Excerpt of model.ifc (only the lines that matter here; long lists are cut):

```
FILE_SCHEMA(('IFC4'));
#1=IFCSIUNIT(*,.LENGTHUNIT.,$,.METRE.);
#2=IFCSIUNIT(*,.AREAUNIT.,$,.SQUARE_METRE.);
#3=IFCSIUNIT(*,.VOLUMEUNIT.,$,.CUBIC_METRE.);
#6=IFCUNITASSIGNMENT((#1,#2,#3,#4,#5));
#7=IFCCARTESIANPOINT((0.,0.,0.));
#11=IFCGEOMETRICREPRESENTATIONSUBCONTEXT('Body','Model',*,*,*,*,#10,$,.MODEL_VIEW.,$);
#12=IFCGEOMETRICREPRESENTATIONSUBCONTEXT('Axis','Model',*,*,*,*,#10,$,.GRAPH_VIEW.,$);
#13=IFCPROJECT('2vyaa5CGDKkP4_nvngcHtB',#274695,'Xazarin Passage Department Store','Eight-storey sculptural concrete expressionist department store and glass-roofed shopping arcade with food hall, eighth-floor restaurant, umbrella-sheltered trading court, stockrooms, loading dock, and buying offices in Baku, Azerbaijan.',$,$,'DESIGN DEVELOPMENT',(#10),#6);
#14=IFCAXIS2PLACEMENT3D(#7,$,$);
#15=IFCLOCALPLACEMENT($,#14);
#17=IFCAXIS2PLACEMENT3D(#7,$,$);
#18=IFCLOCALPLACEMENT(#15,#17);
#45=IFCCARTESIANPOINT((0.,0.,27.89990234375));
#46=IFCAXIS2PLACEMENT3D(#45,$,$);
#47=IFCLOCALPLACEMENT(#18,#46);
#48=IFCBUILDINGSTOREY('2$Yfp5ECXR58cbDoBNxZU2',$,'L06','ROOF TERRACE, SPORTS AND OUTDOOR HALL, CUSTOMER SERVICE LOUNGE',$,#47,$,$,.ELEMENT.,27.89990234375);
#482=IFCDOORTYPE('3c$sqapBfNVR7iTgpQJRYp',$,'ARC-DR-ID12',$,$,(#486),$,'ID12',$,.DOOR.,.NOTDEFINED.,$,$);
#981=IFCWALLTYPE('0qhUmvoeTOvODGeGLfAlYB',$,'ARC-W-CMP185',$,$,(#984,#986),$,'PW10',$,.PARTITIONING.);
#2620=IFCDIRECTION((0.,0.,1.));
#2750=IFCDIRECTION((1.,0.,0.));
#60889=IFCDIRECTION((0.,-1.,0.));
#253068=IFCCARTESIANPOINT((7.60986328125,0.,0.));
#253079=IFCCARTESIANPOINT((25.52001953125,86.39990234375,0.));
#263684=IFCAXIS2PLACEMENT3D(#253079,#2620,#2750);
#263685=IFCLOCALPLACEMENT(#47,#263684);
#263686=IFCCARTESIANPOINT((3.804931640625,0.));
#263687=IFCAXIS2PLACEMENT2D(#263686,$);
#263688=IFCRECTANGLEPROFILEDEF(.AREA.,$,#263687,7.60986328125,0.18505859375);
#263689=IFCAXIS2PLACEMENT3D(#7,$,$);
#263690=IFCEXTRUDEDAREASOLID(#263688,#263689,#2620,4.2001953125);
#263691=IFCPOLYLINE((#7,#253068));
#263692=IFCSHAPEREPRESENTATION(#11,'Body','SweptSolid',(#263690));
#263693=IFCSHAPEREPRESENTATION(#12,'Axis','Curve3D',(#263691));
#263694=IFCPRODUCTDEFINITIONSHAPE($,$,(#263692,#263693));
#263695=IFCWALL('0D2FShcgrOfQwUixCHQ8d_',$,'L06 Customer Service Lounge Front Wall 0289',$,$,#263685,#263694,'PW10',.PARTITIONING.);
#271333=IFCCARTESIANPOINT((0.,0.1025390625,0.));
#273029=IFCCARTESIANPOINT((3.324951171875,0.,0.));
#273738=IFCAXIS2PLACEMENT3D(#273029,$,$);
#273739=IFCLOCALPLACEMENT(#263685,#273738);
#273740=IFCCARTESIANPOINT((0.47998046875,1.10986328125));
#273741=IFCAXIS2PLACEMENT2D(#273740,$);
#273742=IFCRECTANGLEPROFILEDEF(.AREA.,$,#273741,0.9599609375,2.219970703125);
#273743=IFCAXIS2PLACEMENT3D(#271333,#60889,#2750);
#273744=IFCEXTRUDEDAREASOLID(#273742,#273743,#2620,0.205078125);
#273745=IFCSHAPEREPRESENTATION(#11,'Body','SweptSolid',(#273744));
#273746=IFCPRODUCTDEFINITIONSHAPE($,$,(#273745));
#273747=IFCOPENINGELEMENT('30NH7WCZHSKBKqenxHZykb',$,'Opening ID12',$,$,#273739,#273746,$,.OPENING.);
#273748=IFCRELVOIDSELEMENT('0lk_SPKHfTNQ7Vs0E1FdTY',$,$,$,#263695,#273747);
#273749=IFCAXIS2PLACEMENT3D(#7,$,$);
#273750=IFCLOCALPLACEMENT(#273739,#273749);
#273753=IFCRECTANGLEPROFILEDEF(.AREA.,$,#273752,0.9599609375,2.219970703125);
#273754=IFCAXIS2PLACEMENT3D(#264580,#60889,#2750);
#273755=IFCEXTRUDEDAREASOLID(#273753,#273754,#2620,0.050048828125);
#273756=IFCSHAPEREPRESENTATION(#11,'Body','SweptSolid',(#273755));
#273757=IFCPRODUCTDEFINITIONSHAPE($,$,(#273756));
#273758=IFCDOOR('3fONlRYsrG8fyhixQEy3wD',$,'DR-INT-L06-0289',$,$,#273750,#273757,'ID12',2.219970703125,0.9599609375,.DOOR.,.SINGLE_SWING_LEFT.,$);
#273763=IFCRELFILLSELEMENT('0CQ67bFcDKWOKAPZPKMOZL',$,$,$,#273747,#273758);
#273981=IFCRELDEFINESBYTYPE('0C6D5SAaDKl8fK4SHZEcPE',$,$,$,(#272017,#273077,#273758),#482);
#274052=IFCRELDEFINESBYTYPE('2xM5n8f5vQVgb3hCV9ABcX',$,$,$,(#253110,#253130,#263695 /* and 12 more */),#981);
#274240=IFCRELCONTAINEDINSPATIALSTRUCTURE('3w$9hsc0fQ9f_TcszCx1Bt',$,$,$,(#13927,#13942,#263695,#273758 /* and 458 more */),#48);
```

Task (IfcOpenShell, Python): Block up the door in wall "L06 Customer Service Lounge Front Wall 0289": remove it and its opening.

```python
import ifcopenshell
import ifcopenshell.api.feature
import ifcopenshell.api.root
import ifcopenshell.geom
import ifcopenshell.util.shape

model = ifcopenshell.open("model.ifc")
settings = ifcopenshell.geom.settings()


def volume(element):
    """Net volume in cubic metres, openings subtracted."""
    shape = ifcopenshell.geom.create_shape(settings, element)
    return ifcopenshell.util.shape.get_volume(shape.geometry)


door = model.by_guid("3fONlRYsrG8fyhixQEy3wD")
opening = door.FillsVoids[0].RelatingOpeningElement
wall = opening.VoidsElements[0].RelatingBuildingElement
before = volume(wall)

ifcopenshell.api.root.remove_product(model, product=door)
ifcopenshell.api.feature.remove_feature(model, feature=opening)

after = volume(wall)

print(f"wall volume {before:.3f} -> {after:.3f} m3")

model.write("model_edited.ifc")
```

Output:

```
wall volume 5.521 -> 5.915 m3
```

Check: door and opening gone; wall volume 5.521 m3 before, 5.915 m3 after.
